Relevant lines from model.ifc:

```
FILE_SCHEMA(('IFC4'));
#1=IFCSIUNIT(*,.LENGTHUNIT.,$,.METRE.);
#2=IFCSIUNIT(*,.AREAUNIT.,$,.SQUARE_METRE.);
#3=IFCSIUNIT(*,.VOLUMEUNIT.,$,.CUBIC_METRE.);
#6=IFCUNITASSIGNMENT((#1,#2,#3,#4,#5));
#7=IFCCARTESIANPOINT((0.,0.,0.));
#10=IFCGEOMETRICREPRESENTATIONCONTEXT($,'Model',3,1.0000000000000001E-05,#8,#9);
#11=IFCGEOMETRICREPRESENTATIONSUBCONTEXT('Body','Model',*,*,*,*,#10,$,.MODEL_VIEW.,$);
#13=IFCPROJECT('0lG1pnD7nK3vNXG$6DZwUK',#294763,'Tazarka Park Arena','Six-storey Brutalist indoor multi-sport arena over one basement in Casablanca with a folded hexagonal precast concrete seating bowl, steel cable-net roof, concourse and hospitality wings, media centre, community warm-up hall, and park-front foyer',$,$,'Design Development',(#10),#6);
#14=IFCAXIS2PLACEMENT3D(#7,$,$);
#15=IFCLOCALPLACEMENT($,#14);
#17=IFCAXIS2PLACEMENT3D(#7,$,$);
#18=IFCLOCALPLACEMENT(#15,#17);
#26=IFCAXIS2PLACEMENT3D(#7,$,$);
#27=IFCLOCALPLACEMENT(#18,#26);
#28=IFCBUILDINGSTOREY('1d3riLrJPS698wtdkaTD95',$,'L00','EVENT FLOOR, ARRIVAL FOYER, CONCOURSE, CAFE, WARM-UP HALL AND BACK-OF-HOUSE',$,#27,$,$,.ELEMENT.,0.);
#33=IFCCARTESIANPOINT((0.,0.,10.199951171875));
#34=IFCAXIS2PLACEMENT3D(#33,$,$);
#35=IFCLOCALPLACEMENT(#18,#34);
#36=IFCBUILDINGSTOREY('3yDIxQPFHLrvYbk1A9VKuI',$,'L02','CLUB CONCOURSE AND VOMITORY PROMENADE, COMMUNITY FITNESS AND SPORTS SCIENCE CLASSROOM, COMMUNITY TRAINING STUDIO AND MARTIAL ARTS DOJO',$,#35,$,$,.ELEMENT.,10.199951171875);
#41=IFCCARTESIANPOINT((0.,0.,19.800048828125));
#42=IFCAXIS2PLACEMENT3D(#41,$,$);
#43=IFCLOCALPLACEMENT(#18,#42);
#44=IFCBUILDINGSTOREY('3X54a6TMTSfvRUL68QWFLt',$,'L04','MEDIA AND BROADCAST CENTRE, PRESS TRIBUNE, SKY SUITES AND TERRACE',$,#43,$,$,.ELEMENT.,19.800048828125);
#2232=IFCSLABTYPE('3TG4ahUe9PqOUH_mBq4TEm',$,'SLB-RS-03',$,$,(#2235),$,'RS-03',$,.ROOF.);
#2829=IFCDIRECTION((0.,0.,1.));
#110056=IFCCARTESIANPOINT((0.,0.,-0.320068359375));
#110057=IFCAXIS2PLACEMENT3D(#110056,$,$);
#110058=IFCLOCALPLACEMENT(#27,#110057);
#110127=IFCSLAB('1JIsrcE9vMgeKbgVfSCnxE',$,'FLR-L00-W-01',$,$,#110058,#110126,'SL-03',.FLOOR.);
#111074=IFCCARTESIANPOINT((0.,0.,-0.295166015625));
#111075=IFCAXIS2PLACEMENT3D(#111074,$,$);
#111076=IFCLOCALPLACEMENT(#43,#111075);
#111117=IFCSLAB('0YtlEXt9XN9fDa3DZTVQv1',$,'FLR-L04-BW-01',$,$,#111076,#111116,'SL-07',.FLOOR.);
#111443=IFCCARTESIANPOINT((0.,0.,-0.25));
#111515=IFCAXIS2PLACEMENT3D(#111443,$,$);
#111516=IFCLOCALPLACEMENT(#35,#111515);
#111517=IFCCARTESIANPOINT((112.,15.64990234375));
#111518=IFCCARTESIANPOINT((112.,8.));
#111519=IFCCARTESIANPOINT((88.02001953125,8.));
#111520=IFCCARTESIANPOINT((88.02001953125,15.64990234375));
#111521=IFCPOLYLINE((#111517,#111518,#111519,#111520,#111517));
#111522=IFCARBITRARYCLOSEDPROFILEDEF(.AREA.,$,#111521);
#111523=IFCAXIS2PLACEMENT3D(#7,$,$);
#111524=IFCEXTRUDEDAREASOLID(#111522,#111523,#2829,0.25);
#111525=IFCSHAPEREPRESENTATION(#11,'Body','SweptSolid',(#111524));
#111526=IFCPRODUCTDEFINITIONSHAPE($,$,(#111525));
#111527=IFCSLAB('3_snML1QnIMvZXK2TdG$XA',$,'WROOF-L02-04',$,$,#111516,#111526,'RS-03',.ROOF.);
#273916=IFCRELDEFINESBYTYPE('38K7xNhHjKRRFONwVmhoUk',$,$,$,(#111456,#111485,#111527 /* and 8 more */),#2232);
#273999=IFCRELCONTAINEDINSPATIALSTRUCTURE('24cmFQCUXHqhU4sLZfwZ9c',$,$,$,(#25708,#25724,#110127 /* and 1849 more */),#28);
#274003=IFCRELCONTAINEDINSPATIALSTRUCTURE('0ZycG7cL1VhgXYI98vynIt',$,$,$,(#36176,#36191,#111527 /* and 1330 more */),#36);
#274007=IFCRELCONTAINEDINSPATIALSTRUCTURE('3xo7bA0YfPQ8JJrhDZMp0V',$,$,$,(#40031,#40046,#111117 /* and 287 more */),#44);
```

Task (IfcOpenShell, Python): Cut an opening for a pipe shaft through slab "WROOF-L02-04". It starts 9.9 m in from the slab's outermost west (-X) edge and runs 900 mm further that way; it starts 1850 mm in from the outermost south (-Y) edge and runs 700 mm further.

```python
import numpy as np
import ifcopenshell
import ifcopenshell.api.feature
import ifcopenshell.api.geometry
import ifcopenshell.api.root
import ifcopenshell.geom
import ifcopenshell.util.placement
import ifcopenshell.util.representation
import ifcopenshell.util.shape
import ifcopenshell.util.unit

model = ifcopenshell.open("model.ifc")
unit_scale = ifcopenshell.util.unit.calculate_unit_scale(model)
settings = ifcopenshell.geom.settings()


def volume(element):
    """Net volume in cubic metres, openings subtracted."""
    shape = ifcopenshell.geom.create_shape(settings, element)
    return ifcopenshell.util.shape.get_volume(shape.geometry)


slab = model.by_guid("3_snML1QnIMvZXK2TdG$XA")
before = volume(slab)

# Extent in the slab's own axes, in metres. The edges named are its -X and -Y sides.
slab_shape = ifcopenshell.geom.create_shape(settings, slab)
vertices = ifcopenshell.util.shape.get_vertices(slab_shape.geometry)
x_min, y_min, bottom = vertices.min(axis=0)
top = vertices[:, 2].max()

opening = ifcopenshell.api.root.create_entity(model, ifc_class="IfcOpeningElement", name="Pipe shaft opening", predefined_type="OPENING")
context = ifcopenshell.util.representation.get_context(model, "Model", "Body", "MODEL_VIEW")
width, depth = 0.9, 0.7
outline = [(0.0, 0.0), (width, 0.0), (width, depth), (0.0, depth), (0.0, 0.0)]
# Overshoot both faces by 50 mm so the cut is clean.
shape = ifcopenshell.api.geometry.add_slab_representation(
    model, context=context, depth=top - bottom + 0.1, polyline=outline
)
ifcopenshell.api.geometry.assign_representation(model, product=opening, representation=shape)

matrix = ifcopenshell.util.placement.get_local_placement(slab.ObjectPlacement)
matrix[:, 3] = matrix @ np.append(np.array([x_min + 9.9, y_min + 1.85, bottom - 0.05]) / unit_scale, 1.0)
ifcopenshell.api.geometry.edit_object_placement(model, product=opening, matrix=matrix, is_si=False)
ifcopenshell.api.feature.add_feature(model, feature=opening, element=slab)

after = volume(slab)

print(f"slab volume {before:.3f} -> {after:.3f} m3")

model.write("model-out.ifc")
```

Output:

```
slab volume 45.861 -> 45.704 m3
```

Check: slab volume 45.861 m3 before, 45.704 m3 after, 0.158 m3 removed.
